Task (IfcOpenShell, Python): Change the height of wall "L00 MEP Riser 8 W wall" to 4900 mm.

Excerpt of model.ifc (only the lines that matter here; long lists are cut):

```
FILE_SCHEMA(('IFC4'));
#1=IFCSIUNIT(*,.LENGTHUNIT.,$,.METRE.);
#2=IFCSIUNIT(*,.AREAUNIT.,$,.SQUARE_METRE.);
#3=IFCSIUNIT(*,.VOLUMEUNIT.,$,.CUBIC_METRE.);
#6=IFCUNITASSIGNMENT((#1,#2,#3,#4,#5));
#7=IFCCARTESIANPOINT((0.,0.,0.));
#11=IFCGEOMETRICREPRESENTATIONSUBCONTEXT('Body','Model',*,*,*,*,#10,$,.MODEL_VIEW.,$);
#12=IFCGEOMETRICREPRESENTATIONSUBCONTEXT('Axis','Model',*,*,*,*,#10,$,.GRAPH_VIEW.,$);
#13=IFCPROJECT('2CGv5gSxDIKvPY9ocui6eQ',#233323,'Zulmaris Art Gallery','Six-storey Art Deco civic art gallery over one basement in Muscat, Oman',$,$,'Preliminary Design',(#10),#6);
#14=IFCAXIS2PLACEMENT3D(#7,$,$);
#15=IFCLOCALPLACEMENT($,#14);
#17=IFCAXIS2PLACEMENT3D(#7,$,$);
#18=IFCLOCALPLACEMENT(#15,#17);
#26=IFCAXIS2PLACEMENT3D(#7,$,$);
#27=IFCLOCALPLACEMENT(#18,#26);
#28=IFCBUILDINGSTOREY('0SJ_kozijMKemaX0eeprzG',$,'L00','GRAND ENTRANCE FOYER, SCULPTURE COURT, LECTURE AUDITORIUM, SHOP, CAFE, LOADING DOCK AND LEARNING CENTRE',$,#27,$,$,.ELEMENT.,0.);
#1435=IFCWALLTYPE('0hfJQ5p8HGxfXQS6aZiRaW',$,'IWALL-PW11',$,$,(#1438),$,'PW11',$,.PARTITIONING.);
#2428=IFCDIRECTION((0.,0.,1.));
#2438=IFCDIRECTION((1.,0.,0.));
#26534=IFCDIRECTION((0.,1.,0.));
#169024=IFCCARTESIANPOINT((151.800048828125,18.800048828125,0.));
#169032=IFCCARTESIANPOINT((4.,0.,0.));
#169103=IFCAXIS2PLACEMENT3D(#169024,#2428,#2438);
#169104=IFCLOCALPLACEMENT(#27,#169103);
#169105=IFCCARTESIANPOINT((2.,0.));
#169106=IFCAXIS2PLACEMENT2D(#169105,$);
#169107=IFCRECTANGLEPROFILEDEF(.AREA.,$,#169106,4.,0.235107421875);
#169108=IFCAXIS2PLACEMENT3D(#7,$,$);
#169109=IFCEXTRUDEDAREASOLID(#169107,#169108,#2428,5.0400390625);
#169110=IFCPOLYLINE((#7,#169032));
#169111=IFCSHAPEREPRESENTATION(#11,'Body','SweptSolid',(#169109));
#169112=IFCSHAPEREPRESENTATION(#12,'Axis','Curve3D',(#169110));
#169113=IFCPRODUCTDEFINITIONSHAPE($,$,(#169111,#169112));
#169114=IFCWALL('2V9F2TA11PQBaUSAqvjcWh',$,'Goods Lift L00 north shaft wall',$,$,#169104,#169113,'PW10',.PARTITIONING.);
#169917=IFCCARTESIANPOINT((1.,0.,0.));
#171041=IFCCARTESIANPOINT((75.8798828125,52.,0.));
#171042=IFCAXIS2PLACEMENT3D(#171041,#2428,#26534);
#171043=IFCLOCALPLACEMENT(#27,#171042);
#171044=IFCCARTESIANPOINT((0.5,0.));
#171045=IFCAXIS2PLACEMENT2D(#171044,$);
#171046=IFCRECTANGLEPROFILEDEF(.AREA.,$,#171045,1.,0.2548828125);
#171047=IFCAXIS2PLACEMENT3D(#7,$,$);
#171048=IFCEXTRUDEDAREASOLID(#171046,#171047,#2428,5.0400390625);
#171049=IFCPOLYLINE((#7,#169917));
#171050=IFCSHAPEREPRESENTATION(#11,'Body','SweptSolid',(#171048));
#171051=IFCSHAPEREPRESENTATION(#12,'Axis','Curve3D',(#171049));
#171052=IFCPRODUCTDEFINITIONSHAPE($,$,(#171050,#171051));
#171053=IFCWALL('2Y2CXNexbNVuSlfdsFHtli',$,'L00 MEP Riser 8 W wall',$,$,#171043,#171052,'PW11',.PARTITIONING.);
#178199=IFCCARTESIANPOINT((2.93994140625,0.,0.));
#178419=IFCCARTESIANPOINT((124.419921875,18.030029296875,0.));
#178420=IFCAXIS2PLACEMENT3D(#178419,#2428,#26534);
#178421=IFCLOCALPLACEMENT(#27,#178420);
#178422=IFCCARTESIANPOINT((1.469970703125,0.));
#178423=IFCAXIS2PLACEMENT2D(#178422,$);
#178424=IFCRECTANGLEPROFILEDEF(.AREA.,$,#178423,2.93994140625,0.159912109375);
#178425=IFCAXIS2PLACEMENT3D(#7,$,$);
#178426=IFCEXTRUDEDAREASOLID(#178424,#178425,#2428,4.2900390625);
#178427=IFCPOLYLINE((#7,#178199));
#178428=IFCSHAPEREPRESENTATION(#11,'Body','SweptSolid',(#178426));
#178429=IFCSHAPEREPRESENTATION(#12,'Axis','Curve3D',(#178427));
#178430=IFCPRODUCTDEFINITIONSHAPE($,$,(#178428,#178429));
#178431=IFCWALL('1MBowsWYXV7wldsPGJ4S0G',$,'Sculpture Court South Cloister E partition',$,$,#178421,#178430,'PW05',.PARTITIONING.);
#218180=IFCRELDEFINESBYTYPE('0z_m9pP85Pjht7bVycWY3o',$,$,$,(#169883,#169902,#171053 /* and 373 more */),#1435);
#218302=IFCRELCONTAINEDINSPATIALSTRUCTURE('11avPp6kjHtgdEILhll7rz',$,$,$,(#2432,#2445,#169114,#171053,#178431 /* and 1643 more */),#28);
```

```python
import ifcopenshell
import ifcopenshell.geom
import ifcopenshell.util.representation
import ifcopenshell.util.shape
import ifcopenshell.util.unit

model = ifcopenshell.open("model.ifc")
unit_scale = ifcopenshell.util.unit.calculate_unit_scale(model)
settings = ifcopenshell.geom.settings()


def volume(element):
    """Net volume in cubic metres, openings subtracted."""
    shape = ifcopenshell.geom.create_shape(settings, element)
    return ifcopenshell.util.shape.get_volume(shape.geometry)


wall = model.by_guid("2Y2CXNexbNVuSlfdsFHtli")
before = volume(wall)

body = ifcopenshell.util.representation.get_representation(wall, "Model", "Body")
solid = body.Items[0]
old_height = solid.Depth
solid.Depth = 4.9 / unit_scale
after = volume(wall)

print(f"height {old_height:g} -> {solid.Depth:g}, volume {before:.3f} -> {after:.3f} m3")

model.write("model_edited.ifc")
```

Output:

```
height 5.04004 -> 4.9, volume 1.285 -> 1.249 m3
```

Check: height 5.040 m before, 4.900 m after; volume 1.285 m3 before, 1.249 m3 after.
